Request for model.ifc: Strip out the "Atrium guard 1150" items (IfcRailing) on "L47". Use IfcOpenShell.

First a look at what the model holds.

```python
import ifcopenshell
import ifcopenshell.util.element

model = ifcopenshell.open("model.ifc")
print(model.schema)
storey = next(s for s in model.by_type("IfcBuildingStorey") if s.Name == "L47")
railings = [e for e in ifcopenshell.util.element.get_decomposition(storey) if e.is_a("IfcRailing")]
seen = {}
for e in railings:
    element_type = ifcopenshell.util.element.get_type(e)
    name = element_type.Name if element_type not in (None, e) else None
    seen[name] = seen.get(name, 0) + 1
for name, count in sorted(seen.items(), key=str):
    print(count, "x", name)
```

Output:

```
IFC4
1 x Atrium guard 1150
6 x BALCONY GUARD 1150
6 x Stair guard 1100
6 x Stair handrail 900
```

```python
import ifcopenshell
import ifcopenshell.api.root
import ifcopenshell.util.element

model = ifcopenshell.open("model.ifc")

storey = next(s for s in model.by_type("IfcBuildingStorey") if s.Name == "L47")
railings = [e for e in ifcopenshell.util.element.get_decomposition(storey) if e.is_a("IfcRailing")]
targets = [e for e in railings if (t := ifcopenshell.util.element.get_type(e)) not in (None, e) and t.Name == "Atrium guard 1150"]

for e in targets:
    ifcopenshell.api.root.remove_product(model, product=e)
print(len(targets), "removed")

model.write("model_rev.ifc")
```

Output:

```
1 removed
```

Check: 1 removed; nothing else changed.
